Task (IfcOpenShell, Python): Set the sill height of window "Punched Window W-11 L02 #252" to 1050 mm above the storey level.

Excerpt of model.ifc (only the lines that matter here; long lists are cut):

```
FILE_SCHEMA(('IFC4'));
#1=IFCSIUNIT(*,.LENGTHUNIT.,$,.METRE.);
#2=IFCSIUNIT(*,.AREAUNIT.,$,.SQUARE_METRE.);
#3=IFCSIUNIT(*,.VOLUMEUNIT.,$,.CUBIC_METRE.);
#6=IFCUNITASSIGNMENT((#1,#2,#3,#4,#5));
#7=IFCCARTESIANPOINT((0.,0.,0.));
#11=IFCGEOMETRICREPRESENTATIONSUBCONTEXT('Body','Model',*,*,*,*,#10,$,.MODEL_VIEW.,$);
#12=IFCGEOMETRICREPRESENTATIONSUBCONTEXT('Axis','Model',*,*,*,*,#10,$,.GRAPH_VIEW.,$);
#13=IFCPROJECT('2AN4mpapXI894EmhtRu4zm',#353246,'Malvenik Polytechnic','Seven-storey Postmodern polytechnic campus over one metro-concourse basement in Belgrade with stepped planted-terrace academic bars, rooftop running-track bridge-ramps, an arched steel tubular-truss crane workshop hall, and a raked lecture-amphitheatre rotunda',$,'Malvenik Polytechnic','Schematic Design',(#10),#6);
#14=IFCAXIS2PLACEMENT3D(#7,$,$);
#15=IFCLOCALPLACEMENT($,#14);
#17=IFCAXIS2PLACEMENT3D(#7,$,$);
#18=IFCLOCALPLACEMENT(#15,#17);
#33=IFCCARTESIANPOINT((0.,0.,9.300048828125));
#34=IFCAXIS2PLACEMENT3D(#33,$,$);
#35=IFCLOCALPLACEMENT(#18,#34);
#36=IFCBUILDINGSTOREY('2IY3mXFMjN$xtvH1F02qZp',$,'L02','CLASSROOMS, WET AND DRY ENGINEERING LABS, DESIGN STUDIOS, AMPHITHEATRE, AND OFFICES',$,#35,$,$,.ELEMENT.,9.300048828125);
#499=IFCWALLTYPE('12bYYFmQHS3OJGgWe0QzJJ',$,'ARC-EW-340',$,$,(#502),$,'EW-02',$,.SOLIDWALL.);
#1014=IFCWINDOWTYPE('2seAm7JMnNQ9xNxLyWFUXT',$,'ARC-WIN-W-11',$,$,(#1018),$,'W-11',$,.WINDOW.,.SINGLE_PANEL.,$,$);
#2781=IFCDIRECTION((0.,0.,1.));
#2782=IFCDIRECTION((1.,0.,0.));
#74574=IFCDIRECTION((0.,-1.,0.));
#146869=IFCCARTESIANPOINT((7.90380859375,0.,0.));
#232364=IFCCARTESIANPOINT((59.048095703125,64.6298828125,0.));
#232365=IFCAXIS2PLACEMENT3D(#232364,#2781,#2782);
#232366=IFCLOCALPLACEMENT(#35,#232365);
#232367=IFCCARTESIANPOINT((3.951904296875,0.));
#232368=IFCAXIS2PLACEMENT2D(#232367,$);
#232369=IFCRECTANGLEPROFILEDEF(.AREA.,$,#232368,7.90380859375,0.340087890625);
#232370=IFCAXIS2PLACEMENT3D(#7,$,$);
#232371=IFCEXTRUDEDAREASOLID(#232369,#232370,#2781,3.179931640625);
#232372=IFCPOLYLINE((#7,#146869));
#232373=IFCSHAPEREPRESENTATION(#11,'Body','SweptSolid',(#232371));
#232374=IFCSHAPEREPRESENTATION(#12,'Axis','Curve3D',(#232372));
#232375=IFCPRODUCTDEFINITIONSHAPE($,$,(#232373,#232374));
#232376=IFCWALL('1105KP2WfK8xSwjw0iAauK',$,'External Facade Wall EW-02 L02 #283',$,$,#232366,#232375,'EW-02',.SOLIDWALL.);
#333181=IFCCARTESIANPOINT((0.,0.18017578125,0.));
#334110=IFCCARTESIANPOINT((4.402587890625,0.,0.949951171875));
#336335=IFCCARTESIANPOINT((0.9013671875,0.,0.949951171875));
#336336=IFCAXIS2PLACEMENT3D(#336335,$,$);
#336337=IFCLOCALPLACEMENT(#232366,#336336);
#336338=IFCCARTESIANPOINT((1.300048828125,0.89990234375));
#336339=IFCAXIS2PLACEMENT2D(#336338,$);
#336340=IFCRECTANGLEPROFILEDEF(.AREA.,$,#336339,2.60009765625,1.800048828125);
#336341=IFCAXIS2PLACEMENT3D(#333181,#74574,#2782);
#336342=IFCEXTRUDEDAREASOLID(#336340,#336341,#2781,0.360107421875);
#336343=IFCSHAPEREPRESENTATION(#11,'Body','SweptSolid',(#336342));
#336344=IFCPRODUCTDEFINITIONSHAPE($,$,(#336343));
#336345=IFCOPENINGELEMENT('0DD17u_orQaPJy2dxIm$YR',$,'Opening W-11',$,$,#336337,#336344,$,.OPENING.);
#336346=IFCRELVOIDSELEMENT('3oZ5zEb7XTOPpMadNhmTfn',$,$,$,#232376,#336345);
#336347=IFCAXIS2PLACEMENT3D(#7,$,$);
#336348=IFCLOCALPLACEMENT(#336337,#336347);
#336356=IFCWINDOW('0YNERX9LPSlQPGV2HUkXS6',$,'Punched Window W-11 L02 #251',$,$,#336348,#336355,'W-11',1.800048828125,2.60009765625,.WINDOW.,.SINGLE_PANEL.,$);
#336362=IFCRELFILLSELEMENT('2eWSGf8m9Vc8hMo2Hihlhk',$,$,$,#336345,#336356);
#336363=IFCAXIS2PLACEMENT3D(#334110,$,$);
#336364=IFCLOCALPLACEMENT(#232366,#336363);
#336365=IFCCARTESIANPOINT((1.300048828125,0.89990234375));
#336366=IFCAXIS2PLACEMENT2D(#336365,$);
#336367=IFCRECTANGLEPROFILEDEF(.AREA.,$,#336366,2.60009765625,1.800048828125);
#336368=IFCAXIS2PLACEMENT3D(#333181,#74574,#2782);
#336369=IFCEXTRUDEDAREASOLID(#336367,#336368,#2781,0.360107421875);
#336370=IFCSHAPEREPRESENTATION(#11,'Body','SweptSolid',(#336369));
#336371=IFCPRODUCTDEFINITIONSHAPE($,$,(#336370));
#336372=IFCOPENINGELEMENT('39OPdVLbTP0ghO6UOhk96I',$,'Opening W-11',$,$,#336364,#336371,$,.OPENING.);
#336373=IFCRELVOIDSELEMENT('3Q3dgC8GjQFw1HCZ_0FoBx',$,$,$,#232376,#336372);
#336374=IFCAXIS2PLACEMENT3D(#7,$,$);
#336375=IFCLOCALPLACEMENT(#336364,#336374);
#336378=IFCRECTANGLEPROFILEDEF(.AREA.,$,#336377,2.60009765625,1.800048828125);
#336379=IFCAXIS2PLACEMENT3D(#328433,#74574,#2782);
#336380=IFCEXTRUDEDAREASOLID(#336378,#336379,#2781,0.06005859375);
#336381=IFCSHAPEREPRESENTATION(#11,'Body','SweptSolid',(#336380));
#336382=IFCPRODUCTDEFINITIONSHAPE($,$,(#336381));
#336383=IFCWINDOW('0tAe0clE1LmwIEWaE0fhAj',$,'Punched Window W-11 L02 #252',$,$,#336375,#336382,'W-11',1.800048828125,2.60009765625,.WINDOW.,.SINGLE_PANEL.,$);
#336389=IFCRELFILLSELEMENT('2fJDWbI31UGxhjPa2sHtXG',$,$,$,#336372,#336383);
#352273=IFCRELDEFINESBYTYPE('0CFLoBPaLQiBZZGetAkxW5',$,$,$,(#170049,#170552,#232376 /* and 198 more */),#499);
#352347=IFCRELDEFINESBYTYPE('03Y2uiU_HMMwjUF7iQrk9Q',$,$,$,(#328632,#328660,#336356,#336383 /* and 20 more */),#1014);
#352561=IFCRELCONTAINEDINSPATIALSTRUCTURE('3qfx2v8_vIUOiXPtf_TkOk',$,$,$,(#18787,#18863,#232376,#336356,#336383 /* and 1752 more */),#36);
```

```python
import numpy as np
import ifcopenshell
import ifcopenshell.api.geometry
import ifcopenshell.geom
import ifcopenshell.util.element
import ifcopenshell.util.placement
import ifcopenshell.util.shape
import ifcopenshell.util.unit

model = ifcopenshell.open("model.ifc")
unit_scale = ifcopenshell.util.unit.calculate_unit_scale(model)

window = model.by_id(336383)
opening = window.FillsVoids[0].RelatingOpeningElement
storey = ifcopenshell.util.element.get_container(window, ifc_class="IfcBuildingStorey")
level = ifcopenshell.util.placement.get_local_placement(storey.ObjectPlacement)[2, 3]

# The opening's origin need not be at the sill, so measure its lowest point.
shape = ifcopenshell.geom.create_shape(ifcopenshell.geom.settings(), opening)
bottom = ifcopenshell.util.shape.get_shape_bottom_elevation(shape, shape.geometry) / unit_scale
dz = level + 1.05 - bottom

shift = np.array([0.0, 0.0, dz])
# The window is placed relative to its opening, so it follows when the opening moves.
matrix = ifcopenshell.util.placement.get_local_placement(opening.ObjectPlacement)
matrix[:3, 3] += shift
ifcopenshell.api.geometry.edit_object_placement(
    model, product=opening, matrix=matrix, is_si=False, should_transform_children=True
)

print(f"moved by {dz * unit_scale:+.3f} m")

model.write("model_v2.ifc")
```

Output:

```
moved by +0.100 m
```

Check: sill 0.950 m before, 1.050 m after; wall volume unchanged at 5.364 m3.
